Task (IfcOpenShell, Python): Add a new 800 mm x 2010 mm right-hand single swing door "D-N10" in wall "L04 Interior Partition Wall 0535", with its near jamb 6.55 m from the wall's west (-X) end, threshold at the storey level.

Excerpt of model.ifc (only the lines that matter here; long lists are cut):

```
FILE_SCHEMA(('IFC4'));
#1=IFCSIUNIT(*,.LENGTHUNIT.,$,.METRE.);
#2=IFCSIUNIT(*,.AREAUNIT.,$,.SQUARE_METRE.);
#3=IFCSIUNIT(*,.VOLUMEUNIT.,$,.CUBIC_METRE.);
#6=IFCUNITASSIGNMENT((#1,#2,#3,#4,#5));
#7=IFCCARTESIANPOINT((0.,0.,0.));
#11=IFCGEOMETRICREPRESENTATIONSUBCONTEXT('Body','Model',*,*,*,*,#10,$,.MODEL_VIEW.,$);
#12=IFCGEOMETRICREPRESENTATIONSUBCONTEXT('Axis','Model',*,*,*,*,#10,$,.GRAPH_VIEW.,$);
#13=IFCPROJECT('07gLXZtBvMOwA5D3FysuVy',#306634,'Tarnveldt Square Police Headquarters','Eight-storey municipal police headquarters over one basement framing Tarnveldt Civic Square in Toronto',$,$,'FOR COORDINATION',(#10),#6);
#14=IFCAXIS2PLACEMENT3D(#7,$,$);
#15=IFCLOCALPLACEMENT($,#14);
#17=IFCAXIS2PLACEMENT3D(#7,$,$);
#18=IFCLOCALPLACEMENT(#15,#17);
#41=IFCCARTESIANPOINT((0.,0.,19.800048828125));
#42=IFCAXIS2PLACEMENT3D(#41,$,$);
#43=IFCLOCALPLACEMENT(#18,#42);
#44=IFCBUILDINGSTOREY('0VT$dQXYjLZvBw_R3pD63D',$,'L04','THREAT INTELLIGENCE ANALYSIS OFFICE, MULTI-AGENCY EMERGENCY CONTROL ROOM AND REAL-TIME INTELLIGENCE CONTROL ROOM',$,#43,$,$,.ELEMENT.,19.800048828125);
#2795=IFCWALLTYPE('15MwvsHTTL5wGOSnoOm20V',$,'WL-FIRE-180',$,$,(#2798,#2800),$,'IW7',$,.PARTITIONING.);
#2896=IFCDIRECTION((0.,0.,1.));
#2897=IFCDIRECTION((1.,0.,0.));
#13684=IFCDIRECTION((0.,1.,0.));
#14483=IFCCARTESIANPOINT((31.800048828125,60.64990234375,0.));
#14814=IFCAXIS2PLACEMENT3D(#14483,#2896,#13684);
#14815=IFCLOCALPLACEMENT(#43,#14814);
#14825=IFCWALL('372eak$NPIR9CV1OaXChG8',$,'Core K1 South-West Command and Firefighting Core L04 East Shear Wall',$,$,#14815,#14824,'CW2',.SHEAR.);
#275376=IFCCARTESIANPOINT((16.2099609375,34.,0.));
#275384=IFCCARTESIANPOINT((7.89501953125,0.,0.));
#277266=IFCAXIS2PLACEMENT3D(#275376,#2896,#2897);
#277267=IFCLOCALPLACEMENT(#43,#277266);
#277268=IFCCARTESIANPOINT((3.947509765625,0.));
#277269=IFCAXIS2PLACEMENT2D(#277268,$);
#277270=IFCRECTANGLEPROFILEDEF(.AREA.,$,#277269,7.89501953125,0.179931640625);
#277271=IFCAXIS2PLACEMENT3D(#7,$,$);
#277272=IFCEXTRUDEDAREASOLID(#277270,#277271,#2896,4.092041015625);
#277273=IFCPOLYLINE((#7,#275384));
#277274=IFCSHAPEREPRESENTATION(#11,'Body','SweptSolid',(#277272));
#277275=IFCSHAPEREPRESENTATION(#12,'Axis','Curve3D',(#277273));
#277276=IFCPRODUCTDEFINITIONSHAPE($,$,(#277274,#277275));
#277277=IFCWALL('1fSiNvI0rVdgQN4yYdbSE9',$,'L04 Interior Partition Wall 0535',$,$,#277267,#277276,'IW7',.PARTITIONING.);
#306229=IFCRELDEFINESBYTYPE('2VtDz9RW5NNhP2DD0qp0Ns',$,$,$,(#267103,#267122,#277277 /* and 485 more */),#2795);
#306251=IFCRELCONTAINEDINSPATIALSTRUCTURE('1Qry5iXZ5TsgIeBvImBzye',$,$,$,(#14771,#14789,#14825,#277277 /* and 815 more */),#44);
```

```python
import numpy as np
import ifcopenshell
import ifcopenshell.api.feature
import ifcopenshell.api.geometry
import ifcopenshell.api.root
import ifcopenshell.api.spatial
import ifcopenshell.geom
import ifcopenshell.util.element
import ifcopenshell.util.placement
import ifcopenshell.util.representation
import ifcopenshell.util.shape
import ifcopenshell.util.unit

model = ifcopenshell.open("model.ifc")
unit_scale = ifcopenshell.util.unit.calculate_unit_scale(model)
settings = ifcopenshell.geom.settings()


def volume(element):
    """Net volume in cubic metres, openings subtracted."""
    shape = ifcopenshell.geom.create_shape(settings, element)
    return ifcopenshell.util.shape.get_volume(shape.geometry)


wall = model.by_guid("1fSiNvI0rVdgQN4yYdbSE9")
storey = ifcopenshell.util.element.get_container(wall, ifc_class="IfcBuildingStorey")
context = ifcopenshell.util.representation.get_context(model, "Model", "Body", "MODEL_VIEW")
before = volume(wall)

width, height, from_end, sill = 0.8, 2.01, 6.55, 0.0  # metres

# The wall runs along its own X axis, and the end named is its -X end.
wall_shape = ifcopenshell.geom.create_shape(settings, wall)
x, y, z = ifcopenshell.util.shape.get_vertices(wall_shape.geometry).T
start = x.min() + from_end
face, thickness = float(y.min()), float(y.max() - y.min())
wall_matrix = ifcopenshell.util.placement.get_local_placement(wall.ObjectPlacement)
level = ifcopenshell.util.placement.get_local_placement(storey.ObjectPlacement)[2, 3]


def in_wall(x, y):
    """Placement at x, y metres in the wall's axes, at sill height."""
    matrix = wall_matrix.copy()
    matrix[:, 3] = wall_matrix @ np.array([x / unit_scale, y / unit_scale, 0.0, 1.0])
    matrix[2, 3] = level + sill / unit_scale
    return matrix


# Opening: a box that overshoots both wall faces by 50 mm.
opening = ifcopenshell.api.root.create_entity(model, ifc_class="IfcOpeningElement", predefined_type="OPENING")
box = ifcopenshell.api.geometry.add_wall_representation(
    model, context=context, length=width, height=height, thickness=thickness + 0.1
)
ifcopenshell.api.geometry.assign_representation(model, product=opening, representation=box)
ifcopenshell.api.geometry.edit_object_placement(model, product=opening, matrix=in_wall(start, face - 0.05), is_si=False)
ifcopenshell.api.feature.add_feature(model, feature=opening, element=wall)

door = ifcopenshell.api.root.create_entity(model, ifc_class="IfcDoor", name="D-N10", predefined_type="DOOR")
door.OverallWidth, door.OverallHeight = width / unit_scale, height / unit_scale
door.OperationType = "SINGLE_SWING_RIGHT"
body = ifcopenshell.api.geometry.add_door_representation(
    model,
    context=context,
    overall_width=door.OverallWidth,
    overall_height=door.OverallHeight,
    operation_type="SINGLE_SWING_RIGHT",
    lining_properties={"LiningDepth": thickness / unit_scale, "ThresholdDepth": thickness / unit_scale},
)
ifcopenshell.api.geometry.assign_representation(model, product=door, representation=body)
ifcopenshell.api.spatial.assign_container(model, products=[door], relating_structure=storey)
ifcopenshell.api.feature.add_filling(model, opening=opening, element=door)

# The lining spans the wall, so the door starts at the wall face.
ifcopenshell.api.geometry.edit_object_placement(model, product=door, matrix=in_wall(start, face), is_si=False)

after = volume(wall)

print(f"wall volume {before:.3f} -> {after:.3f} m3")

model.write("model_rev.ifc")
```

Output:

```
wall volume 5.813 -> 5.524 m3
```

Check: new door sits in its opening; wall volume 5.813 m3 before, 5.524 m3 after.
